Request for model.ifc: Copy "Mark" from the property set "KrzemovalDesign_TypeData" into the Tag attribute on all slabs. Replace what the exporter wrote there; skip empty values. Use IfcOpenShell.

First a look at what the model holds.

```python
import ifcopenshell
import ifcopenshell.util.element

model = ifcopenshell.open("model.ifc")
print(model.schema)
slabs = model.by_type("IfcSlab")
print(len(slabs), "slabs")
for e in slabs[:8]:
    source = ifcopenshell.util.element.get_pset(e, "KrzemovalDesign_TypeData", "Mark")
    target = e.Tag
    print(e.id(), repr(source), repr(target), sep=" | ")
```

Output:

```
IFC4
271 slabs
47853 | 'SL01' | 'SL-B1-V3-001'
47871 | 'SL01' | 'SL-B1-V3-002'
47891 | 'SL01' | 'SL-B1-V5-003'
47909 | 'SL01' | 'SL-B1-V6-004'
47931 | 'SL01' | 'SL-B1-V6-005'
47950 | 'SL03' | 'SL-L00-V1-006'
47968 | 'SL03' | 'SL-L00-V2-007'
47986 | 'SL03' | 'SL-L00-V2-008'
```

```python
import ifcopenshell
import ifcopenshell.util.element

model = ifcopenshell.open("model.ifc")

count = 0
for e in model.by_type("IfcSlab"):
    value = ifcopenshell.util.element.get_pset(e, "KrzemovalDesign_TypeData", "Mark")
    current = e.Tag
    if not value or not value.strip() or current == value:
        continue
    e.Tag = value
    count += 1

print(count, "slabs updated")

model.write("model_v2.ifc")
```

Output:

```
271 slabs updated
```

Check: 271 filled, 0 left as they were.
